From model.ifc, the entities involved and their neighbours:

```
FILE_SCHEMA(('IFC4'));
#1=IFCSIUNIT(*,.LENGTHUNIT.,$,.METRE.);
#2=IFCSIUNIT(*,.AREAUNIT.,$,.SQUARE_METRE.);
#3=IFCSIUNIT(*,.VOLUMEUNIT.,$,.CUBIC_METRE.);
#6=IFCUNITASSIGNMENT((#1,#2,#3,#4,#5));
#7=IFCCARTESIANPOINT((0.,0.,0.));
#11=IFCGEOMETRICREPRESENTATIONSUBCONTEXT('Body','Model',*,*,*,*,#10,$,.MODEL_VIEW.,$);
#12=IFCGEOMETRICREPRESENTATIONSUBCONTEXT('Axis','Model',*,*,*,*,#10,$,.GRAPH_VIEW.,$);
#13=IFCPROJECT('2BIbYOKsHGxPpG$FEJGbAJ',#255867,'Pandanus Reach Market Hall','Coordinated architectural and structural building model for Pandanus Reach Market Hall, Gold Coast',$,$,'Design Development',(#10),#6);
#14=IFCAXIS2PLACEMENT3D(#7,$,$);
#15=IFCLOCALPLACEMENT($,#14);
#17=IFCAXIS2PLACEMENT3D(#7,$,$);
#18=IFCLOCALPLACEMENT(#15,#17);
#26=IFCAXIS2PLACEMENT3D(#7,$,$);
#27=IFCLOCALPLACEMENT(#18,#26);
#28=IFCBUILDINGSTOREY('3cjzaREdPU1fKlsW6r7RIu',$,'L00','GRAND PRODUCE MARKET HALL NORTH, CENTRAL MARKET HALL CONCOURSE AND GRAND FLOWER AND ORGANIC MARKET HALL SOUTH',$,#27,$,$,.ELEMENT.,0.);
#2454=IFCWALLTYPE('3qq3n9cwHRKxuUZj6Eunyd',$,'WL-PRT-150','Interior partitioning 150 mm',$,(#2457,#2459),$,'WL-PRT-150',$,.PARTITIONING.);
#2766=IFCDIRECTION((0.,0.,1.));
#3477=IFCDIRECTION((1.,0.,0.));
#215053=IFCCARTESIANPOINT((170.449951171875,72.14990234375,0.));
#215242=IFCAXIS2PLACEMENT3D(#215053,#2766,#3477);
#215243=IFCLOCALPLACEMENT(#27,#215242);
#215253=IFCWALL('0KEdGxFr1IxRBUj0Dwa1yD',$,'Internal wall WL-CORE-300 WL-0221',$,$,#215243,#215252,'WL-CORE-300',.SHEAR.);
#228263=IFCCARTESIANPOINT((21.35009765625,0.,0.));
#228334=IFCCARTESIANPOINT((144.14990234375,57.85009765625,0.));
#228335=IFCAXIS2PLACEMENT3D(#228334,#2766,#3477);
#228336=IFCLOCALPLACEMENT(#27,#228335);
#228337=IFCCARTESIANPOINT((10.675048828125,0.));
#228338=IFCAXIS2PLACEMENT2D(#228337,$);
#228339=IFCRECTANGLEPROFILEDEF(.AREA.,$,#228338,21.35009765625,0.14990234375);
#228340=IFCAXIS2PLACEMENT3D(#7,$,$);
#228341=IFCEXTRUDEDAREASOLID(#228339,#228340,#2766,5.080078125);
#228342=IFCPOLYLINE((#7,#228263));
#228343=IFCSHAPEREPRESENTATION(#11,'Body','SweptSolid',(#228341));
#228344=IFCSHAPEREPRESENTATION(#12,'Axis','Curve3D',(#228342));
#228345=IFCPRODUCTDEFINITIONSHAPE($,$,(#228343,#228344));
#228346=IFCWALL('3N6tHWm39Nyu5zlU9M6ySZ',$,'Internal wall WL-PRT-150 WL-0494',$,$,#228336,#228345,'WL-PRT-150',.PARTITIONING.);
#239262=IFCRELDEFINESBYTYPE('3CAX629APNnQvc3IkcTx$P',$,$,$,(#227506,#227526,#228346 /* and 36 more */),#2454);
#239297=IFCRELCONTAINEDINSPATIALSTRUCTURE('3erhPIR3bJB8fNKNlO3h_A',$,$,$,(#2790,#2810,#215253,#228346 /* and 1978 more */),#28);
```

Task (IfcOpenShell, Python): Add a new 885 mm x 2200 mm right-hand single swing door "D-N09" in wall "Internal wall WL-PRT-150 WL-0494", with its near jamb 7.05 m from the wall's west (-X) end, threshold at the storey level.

```python
import numpy as np
import ifcopenshell
import ifcopenshell.api.feature
import ifcopenshell.api.geometry
import ifcopenshell.api.root
import ifcopenshell.api.spatial
import ifcopenshell.geom
import ifcopenshell.util.element
import ifcopenshell.util.placement
import ifcopenshell.util.representation
import ifcopenshell.util.shape
import ifcopenshell.util.unit

model = ifcopenshell.open("model.ifc")
unit_scale = ifcopenshell.util.unit.calculate_unit_scale(model)
settings = ifcopenshell.geom.settings()


def volume(element):
    """Net volume in cubic metres, openings subtracted."""
    shape = ifcopenshell.geom.create_shape(settings, element)
    return ifcopenshell.util.shape.get_volume(shape.geometry)


wall = model.by_guid("3N6tHWm39Nyu5zlU9M6ySZ")
storey = ifcopenshell.util.element.get_container(wall, ifc_class="IfcBuildingStorey")
context = ifcopenshell.util.representation.get_context(model, "Model", "Body", "MODEL_VIEW")
before = volume(wall)

width, height, from_end, sill = 0.885, 2.2, 7.05, 0.0  # metres

# The wall runs along its own X axis, and the end named is its -X end.
wall_shape = ifcopenshell.geom.create_shape(settings, wall)
x, y, z = ifcopenshell.util.shape.get_vertices(wall_shape.geometry).T
start = x.min() + from_end
face, thickness = float(y.min()), float(y.max() - y.min())
wall_matrix = ifcopenshell.util.placement.get_local_placement(wall.ObjectPlacement)
level = ifcopenshell.util.placement.get_local_placement(storey.ObjectPlacement)[2, 3]


def in_wall(x, y):
    """Placement at x, y metres in the wall's axes, at sill height."""
    matrix = wall_matrix.copy()
    matrix[:, 3] = wall_matrix @ np.array([x / unit_scale, y / unit_scale, 0.0, 1.0])
    matrix[2, 3] = level + sill / unit_scale
    return matrix


# Opening: a box that overshoots both wall faces by 50 mm.
opening = ifcopenshell.api.root.create_entity(model, ifc_class="IfcOpeningElement", predefined_type="OPENING")
box = ifcopenshell.api.geometry.add_wall_representation(
    model, context=context, length=width, height=height, thickness=thickness + 0.1
)
ifcopenshell.api.geometry.assign_representation(model, product=opening, representation=box)
ifcopenshell.api.geometry.edit_object_placement(model, product=opening, matrix=in_wall(start, face - 0.05), is_si=False)
ifcopenshell.api.feature.add_feature(model, feature=opening, element=wall)

door = ifcopenshell.api.root.create_entity(model, ifc_class="IfcDoor", name="D-N09", predefined_type="DOOR")
door.OverallWidth, door.OverallHeight = width / unit_scale, height / unit_scale
door.OperationType = "SINGLE_SWING_RIGHT"
body = ifcopenshell.api.geometry.add_door_representation(
    model,
    context=context,
    overall_width=door.OverallWidth,
    overall_height=door.OverallHeight,
    operation_type="SINGLE_SWING_RIGHT",
    lining_properties={"LiningDepth": thickness / unit_scale, "ThresholdDepth": thickness / unit_scale},
)
ifcopenshell.api.geometry.assign_representation(model, product=door, representation=body)
ifcopenshell.api.spatial.assign_container(model, products=[door], relating_structure=storey)
ifcopenshell.api.feature.add_filling(model, opening=opening, element=door)

# The lining spans the wall, so the door starts at the wall face.
ifcopenshell.api.geometry.edit_object_placement(model, product=door, matrix=in_wall(start, face), is_si=False)

after = volume(wall)

print(f"wall volume {before:.3f} -> {after:.3f} m3")

model.write("model-out.ifc")
```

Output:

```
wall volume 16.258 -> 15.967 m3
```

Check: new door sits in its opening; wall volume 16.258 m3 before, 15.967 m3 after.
